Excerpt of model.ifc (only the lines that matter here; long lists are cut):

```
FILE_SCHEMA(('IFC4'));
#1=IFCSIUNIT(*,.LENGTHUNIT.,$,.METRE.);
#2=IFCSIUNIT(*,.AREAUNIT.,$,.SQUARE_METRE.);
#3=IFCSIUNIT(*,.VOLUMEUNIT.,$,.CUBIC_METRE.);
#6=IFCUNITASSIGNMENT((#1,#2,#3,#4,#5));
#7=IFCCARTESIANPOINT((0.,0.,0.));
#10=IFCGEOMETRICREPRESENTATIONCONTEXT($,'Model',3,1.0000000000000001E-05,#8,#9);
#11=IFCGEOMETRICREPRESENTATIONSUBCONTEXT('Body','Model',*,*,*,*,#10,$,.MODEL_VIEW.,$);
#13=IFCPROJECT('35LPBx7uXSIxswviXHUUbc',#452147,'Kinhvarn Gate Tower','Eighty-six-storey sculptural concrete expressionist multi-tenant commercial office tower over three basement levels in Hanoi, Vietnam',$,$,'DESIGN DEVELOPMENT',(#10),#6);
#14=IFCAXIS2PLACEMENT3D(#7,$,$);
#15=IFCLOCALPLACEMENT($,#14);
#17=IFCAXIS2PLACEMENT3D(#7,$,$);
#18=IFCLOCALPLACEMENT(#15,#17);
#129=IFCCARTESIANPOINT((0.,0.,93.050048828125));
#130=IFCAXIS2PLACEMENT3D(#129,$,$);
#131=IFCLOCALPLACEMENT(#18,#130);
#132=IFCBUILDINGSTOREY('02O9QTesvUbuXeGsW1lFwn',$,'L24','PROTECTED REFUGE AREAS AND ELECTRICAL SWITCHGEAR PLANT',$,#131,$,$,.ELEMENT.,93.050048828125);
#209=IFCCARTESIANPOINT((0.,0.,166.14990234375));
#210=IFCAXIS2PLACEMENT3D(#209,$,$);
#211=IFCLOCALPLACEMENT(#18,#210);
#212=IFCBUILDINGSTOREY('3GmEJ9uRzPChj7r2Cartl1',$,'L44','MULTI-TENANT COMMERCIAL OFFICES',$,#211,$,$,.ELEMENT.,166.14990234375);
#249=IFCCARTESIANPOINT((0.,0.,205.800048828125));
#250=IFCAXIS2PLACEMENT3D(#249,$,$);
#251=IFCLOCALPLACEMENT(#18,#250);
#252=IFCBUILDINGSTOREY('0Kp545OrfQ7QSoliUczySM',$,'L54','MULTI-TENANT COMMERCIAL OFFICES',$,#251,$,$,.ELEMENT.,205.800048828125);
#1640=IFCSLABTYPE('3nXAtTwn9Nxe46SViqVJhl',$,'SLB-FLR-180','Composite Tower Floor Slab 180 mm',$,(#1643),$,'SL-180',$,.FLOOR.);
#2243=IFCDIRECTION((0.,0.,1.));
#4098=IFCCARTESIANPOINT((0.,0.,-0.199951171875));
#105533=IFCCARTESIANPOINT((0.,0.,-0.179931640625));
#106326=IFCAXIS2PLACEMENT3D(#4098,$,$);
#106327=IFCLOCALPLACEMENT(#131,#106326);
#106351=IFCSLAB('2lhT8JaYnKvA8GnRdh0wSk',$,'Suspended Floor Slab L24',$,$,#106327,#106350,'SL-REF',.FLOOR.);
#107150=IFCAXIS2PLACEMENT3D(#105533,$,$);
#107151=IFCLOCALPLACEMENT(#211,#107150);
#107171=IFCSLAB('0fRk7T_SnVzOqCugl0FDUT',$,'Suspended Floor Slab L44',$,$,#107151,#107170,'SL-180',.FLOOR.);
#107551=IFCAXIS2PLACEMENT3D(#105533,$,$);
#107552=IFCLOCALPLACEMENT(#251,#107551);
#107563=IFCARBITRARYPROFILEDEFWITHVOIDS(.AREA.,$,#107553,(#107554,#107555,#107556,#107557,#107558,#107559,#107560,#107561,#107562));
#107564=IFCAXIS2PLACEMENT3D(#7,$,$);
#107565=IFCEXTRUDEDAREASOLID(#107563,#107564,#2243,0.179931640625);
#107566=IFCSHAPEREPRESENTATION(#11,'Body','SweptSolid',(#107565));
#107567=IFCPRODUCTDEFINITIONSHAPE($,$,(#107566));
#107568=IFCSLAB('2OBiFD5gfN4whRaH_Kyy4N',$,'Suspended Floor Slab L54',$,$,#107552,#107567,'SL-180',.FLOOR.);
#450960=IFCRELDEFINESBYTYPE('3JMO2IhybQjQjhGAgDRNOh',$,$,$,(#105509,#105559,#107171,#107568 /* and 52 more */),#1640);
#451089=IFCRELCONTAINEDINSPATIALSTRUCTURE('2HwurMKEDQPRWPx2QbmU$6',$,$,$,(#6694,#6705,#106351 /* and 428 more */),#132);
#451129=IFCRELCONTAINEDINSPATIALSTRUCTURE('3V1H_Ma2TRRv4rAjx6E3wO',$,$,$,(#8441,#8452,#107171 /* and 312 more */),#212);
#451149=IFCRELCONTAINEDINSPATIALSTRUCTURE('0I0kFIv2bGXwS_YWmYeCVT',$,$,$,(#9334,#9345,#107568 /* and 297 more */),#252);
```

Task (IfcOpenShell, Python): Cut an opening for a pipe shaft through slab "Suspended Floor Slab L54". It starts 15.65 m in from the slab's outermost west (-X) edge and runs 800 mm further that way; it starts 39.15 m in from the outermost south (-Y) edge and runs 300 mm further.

```python
import numpy as np
import ifcopenshell
import ifcopenshell.api.feature
import ifcopenshell.api.geometry
import ifcopenshell.api.root
import ifcopenshell.geom
import ifcopenshell.util.placement
import ifcopenshell.util.representation
import ifcopenshell.util.shape
import ifcopenshell.util.unit

model = ifcopenshell.open("model.ifc")
unit_scale = ifcopenshell.util.unit.calculate_unit_scale(model)
settings = ifcopenshell.geom.settings()


def volume(element):
    """Net volume in cubic metres, openings subtracted."""
    shape = ifcopenshell.geom.create_shape(settings, element)
    return ifcopenshell.util.shape.get_volume(shape.geometry)


slab = model.by_guid("2OBiFD5gfN4whRaH_Kyy4N")
before = volume(slab)

# Extent in the slab's own axes, in metres. The edges named are its -X and -Y sides.
slab_shape = ifcopenshell.geom.create_shape(settings, slab)
vertices = ifcopenshell.util.shape.get_vertices(slab_shape.geometry)
x_min, y_min, bottom = vertices.min(axis=0)
top = vertices[:, 2].max()

opening = ifcopenshell.api.root.create_entity(model, ifc_class="IfcOpeningElement", name="Pipe shaft opening", predefined_type="OPENING")
context = ifcopenshell.util.representation.get_context(model, "Model", "Body", "MODEL_VIEW")
width, depth = 0.8, 0.3
outline = [(0.0, 0.0), (width, 0.0), (width, depth), (0.0, depth), (0.0, 0.0)]
# Overshoot both faces by 50 mm so the cut is clean.
shape = ifcopenshell.api.geometry.add_slab_representation(
    model, context=context, depth=top - bottom + 0.1, polyline=outline
)
ifcopenshell.api.geometry.assign_representation(model, product=opening, representation=shape)

matrix = ifcopenshell.util.placement.get_local_placement(slab.ObjectPlacement)
matrix[:, 3] = matrix @ np.append(np.array([x_min + 15.65, y_min + 39.15, bottom - 0.05]) / unit_scale, 1.0)
ifcopenshell.api.geometry.edit_object_placement(model, product=opening, matrix=matrix, is_si=False)
ifcopenshell.api.feature.add_feature(model, feature=opening, element=slab)

after = volume(slab)

print(f"slab volume {before:.3f} -> {after:.3f} m3")

model.write("model-out.ifc")
```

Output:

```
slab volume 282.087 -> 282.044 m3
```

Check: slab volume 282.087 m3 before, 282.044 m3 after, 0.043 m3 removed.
